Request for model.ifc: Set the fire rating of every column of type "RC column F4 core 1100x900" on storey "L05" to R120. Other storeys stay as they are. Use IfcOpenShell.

First a look at what the model holds.

```python
import ifcopenshell
import ifcopenshell.util.element

model = ifcopenshell.open("model.ifc")
print(model.schema)
storey = next(s for s in model.by_type("IfcBuildingStorey") if s.Name == "L05")
columns = [e for e in ifcopenshell.util.element.get_decomposition(storey) if e.is_a("IfcColumn")]
seen = {}
for e in columns:
    element_type = ifcopenshell.util.element.get_type(e)
    key = (element_type.Name if element_type != e and element_type else None, ifcopenshell.util.element.get_pset(e, "Pset_ColumnCommon", "FireRating"))
    seen[key] = seen.get(key, 0) + 1
for (name, value), count in sorted(seen.items(), key=str):
    print(count, "x", name, "|", value)
```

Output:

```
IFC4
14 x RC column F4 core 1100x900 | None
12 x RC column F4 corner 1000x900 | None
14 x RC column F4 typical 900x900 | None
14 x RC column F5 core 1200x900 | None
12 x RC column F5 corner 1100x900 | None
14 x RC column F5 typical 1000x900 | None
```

```python
import ifcopenshell
import ifcopenshell.api.pset
import ifcopenshell.util.element

model = ifcopenshell.open("model.ifc")

storey = next(s for s in model.by_type("IfcBuildingStorey") if s.Name == "L05")
columns = [e for e in ifcopenshell.util.element.get_decomposition(storey) if e.is_a("IfcColumn")]

count = 0
for e in columns:
    element_type = ifcopenshell.util.element.get_type(e)
    if element_type in (None, e) or element_type.Name != "RC column F4 core 1100x900":
        continue
    # add_pset returns the element's existing set when there is one.
    pset = ifcopenshell.api.pset.add_pset(model, product=e, name="Pset_ColumnCommon")
    ifcopenshell.api.pset.edit_pset(model, pset=pset, properties={"FireRating": "R120"})
    count += 1

print(count, "columns updated")

model.write("model_v2.ifc")
```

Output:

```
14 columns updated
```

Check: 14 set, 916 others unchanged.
